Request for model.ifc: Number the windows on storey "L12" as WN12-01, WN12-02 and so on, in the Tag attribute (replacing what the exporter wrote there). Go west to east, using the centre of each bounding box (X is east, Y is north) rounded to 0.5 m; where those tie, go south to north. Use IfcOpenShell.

First a look at what the model holds.

```python
import ifcopenshell
import ifcopenshell.util.element
import ifcopenshell.util.placement

model = ifcopenshell.open("model.ifc")
print(model.schema)
storey = next(s for s in model.by_type("IfcBuildingStorey") if s.Name == "L12")
windows = [e for e in ifcopenshell.util.element.get_decomposition(storey) if e.is_a("IfcWindow")]
for e in sorted(windows, key=lambda e: e.id()):
    origin = ifcopenshell.util.placement.get_local_placement(e.ObjectPlacement)[:3, 3]
    print(e.id(), e.Tag, e.Name, origin.round(2) + 0.0, sep=" | ")
```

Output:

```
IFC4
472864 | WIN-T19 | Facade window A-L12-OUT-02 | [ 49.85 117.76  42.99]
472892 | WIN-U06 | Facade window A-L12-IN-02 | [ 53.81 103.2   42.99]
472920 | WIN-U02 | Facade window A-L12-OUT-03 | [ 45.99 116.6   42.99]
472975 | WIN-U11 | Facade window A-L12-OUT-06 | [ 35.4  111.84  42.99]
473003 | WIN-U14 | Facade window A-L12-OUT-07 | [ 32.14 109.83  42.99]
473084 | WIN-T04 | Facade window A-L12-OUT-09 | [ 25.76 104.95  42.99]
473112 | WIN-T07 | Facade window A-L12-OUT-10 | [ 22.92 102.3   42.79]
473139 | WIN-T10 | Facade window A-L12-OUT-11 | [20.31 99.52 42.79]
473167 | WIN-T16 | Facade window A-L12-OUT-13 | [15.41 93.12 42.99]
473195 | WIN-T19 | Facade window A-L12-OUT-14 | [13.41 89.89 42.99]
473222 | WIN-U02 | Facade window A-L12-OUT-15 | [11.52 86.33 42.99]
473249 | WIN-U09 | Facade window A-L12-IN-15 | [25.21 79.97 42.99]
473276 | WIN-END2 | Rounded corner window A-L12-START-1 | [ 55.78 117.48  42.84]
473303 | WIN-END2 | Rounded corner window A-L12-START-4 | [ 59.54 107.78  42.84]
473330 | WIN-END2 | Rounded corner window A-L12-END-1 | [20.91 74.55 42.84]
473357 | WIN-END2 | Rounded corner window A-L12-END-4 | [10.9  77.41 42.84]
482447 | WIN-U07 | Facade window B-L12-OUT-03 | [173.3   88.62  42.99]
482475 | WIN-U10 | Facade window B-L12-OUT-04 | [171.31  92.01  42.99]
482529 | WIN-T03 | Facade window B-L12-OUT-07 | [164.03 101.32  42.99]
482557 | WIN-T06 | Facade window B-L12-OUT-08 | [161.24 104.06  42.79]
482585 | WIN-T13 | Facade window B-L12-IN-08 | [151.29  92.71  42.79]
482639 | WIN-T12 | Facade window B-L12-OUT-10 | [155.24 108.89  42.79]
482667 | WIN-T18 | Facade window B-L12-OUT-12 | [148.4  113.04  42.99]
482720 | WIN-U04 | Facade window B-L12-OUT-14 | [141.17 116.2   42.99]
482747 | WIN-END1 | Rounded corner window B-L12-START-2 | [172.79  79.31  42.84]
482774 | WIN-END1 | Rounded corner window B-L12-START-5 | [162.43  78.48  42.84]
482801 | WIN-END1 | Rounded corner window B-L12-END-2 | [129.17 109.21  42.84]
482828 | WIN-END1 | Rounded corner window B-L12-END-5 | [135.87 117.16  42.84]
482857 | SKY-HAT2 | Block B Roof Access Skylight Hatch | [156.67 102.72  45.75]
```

```python
import ifcopenshell
import ifcopenshell.geom
import ifcopenshell.util.element
import ifcopenshell.util.shape

model = ifcopenshell.open("model.ifc")
settings = ifcopenshell.geom.settings()
settings.set("use-world-coords", True)


def centre(element):
    shape = ifcopenshell.geom.create_shape(settings, element)
    return ifcopenshell.util.shape.get_bbox_centroid(shape.geometry)


storey = next(s for s in model.by_type("IfcBuildingStorey") if s.Name == "L12")
windows = [e for e in ifcopenshell.util.element.get_decomposition(storey) if e.is_a("IfcWindow")]

# Insertion points can sit at a corner or the storey origin, so sort by the geometry (in metres).
centres = {e: centre(e) for e in windows}
windows.sort(key=lambda e: (round(centres[e][0] / 0.5), centres[e][1]))

for i, e in enumerate(windows, start=1):
    number = f"WN12-{i:02d}"
    e.Tag = number
    print(e.id(), number)

model.write("model_updated.ifc")
```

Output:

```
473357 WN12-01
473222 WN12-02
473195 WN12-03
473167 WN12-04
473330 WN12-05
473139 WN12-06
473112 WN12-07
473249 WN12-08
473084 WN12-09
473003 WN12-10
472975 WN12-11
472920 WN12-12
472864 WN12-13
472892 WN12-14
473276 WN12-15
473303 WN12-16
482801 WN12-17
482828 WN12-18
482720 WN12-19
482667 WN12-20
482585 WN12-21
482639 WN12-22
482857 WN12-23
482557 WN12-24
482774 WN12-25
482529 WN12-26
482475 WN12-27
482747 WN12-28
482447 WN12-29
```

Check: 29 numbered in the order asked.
